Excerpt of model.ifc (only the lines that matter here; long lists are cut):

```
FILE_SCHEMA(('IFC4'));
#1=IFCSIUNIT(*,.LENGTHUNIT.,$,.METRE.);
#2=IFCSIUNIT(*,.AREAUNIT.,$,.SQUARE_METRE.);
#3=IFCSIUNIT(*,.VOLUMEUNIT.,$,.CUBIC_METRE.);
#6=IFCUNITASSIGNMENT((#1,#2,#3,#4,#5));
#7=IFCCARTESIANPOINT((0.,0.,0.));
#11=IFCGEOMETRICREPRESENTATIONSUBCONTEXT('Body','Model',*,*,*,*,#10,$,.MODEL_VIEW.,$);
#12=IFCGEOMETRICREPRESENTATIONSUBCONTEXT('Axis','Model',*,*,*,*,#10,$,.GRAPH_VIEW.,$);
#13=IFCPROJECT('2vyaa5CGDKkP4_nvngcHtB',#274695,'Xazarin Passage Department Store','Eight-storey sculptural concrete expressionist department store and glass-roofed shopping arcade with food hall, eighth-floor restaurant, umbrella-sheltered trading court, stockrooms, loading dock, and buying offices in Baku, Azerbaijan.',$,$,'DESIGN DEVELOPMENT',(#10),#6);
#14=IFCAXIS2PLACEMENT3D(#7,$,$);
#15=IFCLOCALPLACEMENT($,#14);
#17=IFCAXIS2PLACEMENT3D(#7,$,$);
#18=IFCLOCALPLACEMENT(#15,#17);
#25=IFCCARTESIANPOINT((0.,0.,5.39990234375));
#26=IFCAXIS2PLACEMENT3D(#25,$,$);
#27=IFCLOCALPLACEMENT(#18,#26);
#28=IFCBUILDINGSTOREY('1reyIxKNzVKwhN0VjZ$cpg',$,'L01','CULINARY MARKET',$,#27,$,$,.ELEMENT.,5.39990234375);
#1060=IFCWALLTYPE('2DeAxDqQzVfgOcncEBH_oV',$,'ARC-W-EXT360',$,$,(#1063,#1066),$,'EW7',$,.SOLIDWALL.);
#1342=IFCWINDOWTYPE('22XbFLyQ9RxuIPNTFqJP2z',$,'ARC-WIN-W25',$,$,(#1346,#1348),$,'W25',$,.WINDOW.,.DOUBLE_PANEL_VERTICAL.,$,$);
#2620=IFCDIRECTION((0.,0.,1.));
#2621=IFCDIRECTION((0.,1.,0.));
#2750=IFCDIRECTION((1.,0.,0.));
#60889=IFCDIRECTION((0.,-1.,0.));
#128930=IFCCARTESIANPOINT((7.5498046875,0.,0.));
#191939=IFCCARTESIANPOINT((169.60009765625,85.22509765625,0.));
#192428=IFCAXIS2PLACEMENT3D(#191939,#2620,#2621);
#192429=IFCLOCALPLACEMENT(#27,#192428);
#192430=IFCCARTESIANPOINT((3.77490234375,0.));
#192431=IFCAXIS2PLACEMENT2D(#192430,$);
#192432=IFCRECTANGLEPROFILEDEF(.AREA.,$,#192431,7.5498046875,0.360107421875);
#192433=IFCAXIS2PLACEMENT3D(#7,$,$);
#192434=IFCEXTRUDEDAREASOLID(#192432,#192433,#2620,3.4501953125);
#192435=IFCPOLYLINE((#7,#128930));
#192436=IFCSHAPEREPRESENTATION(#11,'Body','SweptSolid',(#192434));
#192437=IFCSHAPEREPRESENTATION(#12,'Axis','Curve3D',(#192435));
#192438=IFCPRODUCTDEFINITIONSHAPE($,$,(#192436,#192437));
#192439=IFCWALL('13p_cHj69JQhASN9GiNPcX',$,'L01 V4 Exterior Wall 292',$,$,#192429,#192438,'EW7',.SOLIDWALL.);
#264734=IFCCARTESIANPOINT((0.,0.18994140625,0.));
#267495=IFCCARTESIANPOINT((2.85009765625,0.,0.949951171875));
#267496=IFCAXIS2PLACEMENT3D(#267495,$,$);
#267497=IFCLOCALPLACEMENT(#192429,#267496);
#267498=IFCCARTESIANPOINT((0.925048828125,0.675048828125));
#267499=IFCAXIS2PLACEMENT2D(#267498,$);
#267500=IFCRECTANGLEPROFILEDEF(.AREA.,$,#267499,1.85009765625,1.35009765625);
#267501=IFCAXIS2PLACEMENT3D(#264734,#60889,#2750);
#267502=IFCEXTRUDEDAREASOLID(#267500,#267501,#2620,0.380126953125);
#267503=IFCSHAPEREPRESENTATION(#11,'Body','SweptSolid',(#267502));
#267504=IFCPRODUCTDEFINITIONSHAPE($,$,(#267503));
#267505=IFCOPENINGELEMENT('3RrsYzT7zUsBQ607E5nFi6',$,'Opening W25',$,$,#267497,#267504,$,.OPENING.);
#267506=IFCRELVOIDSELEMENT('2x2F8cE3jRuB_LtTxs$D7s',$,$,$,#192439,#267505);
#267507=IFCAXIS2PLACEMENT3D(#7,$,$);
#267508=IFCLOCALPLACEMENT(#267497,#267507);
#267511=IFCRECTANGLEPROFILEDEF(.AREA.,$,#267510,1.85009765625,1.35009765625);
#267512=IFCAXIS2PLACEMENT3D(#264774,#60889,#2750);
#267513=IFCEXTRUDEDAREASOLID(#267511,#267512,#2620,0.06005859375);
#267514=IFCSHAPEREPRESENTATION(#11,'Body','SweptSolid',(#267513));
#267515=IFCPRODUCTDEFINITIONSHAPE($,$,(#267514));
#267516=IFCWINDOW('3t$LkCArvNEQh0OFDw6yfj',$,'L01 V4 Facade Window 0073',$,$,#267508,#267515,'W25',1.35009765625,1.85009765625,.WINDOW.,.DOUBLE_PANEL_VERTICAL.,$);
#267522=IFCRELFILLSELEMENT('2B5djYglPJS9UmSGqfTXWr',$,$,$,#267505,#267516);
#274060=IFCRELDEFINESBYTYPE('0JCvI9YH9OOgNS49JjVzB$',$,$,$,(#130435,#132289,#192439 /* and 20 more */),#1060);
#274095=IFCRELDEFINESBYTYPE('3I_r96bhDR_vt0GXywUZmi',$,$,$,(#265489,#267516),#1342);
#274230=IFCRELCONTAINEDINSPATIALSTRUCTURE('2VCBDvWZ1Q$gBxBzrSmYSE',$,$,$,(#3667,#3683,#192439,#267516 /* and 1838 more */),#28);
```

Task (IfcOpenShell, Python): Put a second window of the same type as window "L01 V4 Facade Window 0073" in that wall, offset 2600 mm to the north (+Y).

```python
import ifcopenshell
import ifcopenshell.api.feature
import ifcopenshell.api.geometry
import ifcopenshell.api.root
import ifcopenshell.geom
import ifcopenshell.util.element
import ifcopenshell.util.placement
import ifcopenshell.util.shape
import ifcopenshell.util.unit

model = ifcopenshell.open("model.ifc")
unit_scale = ifcopenshell.util.unit.calculate_unit_scale(model)
settings = ifcopenshell.geom.settings()


def volume(element):
    """Net volume in cubic metres, openings subtracted."""
    shape = ifcopenshell.geom.create_shape(settings, element)
    return ifcopenshell.util.shape.get_volume(shape.geometry)


window = model.by_guid("3t$LkCArvNEQh0OFDw6yfj")
opening = window.FillsVoids[0].RelatingOpeningElement
wall = opening.VoidsElements[0].RelatingBuildingElement
before = volume(wall)
shift = ifcopenshell.util.placement.get_local_placement(wall.ObjectPlacement)[:3, 0] * 2.6 / unit_scale

# copy_class copies the void relationship, type, container and properties, but no geometry.
new_opening = ifcopenshell.api.root.copy_class(model, product=opening)
new_opening.Representation = ifcopenshell.util.element.copy_deep(
    model, opening.Representation, exclude=["IfcGeometricRepresentationContext", "IfcRepresentationMap"]
)
new_window = ifcopenshell.api.root.copy_class(model, product=window)
new_window.Representation = ifcopenshell.util.element.copy_deep(
    model, window.Representation, exclude=["IfcGeometricRepresentationContext", "IfcRepresentationMap"]
)
new_window.Tag = None
ifcopenshell.api.feature.add_filling(model, opening=new_opening, element=new_window)

for old, new in ((opening, new_opening), (window, new_window)):
    matrix = ifcopenshell.util.placement.get_local_placement(old.ObjectPlacement)
    matrix[:3, 3] += shift
    ifcopenshell.api.geometry.edit_object_placement(model, product=new, matrix=matrix, is_si=False)

after = volume(wall)

print(f"wall volume {before:.3f} -> {after:.3f} m3")

model.write("model_edited.ifc")
```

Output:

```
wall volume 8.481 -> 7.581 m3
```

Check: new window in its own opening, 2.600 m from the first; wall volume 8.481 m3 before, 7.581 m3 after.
